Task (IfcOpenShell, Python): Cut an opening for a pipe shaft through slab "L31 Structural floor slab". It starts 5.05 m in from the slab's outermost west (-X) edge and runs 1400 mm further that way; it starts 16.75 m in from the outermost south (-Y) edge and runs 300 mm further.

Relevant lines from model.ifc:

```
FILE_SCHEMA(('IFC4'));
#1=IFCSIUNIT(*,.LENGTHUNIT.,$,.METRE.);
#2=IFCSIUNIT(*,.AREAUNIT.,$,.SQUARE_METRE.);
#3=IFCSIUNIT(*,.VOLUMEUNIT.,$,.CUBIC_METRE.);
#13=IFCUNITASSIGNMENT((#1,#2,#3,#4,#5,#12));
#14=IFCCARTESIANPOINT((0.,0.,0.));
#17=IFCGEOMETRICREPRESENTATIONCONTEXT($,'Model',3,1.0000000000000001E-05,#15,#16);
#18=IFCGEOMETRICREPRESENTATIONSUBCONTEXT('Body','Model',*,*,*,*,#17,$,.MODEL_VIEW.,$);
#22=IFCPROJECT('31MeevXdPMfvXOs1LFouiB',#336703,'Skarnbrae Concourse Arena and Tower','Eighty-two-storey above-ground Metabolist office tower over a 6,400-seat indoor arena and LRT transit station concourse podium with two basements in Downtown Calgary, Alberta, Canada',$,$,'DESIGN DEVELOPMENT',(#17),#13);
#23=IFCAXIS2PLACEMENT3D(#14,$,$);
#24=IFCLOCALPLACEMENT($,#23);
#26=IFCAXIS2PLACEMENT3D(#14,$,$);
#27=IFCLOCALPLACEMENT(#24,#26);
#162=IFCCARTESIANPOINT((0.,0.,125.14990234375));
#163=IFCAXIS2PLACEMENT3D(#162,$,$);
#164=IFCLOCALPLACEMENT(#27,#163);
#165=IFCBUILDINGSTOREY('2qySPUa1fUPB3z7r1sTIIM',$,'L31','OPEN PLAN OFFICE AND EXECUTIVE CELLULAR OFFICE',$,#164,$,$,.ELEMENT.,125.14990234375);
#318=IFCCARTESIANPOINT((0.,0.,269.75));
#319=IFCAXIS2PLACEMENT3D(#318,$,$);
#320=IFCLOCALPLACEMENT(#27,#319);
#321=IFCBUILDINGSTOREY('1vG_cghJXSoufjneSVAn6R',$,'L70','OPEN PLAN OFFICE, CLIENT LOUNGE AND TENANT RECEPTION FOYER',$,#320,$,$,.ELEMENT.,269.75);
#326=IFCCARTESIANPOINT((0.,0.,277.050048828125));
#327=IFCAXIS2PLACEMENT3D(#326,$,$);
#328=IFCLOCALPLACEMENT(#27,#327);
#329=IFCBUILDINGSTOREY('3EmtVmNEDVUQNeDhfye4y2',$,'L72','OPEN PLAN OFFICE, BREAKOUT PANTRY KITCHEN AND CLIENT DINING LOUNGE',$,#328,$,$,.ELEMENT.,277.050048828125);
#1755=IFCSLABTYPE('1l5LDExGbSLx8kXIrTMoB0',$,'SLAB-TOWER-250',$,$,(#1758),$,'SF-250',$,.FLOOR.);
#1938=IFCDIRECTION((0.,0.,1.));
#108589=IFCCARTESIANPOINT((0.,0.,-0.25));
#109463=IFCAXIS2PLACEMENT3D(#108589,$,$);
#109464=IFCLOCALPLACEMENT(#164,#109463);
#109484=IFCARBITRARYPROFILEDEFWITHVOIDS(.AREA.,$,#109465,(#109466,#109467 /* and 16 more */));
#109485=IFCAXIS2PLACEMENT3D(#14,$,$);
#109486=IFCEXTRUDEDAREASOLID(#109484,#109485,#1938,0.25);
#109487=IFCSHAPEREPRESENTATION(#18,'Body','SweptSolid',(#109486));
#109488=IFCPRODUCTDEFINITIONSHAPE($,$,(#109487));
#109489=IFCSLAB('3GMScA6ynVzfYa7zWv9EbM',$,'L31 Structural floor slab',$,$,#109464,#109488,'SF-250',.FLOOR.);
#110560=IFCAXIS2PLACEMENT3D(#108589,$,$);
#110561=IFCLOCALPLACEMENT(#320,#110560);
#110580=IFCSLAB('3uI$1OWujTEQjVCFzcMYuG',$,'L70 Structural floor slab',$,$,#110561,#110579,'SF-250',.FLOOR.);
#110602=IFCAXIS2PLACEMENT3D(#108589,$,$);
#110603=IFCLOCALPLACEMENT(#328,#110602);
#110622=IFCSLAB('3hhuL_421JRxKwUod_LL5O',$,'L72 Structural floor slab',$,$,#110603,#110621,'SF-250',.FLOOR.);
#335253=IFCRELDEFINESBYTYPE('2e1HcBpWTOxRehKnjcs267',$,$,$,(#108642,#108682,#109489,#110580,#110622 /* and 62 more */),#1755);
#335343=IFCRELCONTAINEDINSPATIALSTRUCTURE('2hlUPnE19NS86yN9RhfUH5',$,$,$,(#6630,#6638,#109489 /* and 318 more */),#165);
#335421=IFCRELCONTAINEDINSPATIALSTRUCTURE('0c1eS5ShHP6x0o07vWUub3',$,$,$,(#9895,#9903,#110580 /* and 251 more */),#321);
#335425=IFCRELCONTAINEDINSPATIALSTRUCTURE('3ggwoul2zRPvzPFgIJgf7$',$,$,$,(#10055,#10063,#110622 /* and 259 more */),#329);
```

```python
import numpy as np
import ifcopenshell
import ifcopenshell.api.feature
import ifcopenshell.api.geometry
import ifcopenshell.api.root
import ifcopenshell.geom
import ifcopenshell.util.placement
import ifcopenshell.util.representation
import ifcopenshell.util.shape
import ifcopenshell.util.unit

model = ifcopenshell.open("model.ifc")
unit_scale = ifcopenshell.util.unit.calculate_unit_scale(model)
settings = ifcopenshell.geom.settings()


def volume(element):
    """Net volume in cubic metres, openings subtracted."""
    shape = ifcopenshell.geom.create_shape(settings, element)
    return ifcopenshell.util.shape.get_volume(shape.geometry)


slab = model.by_id(109489)
before = volume(slab)

# Extent in the slab's own axes, in metres. The edges named are its -X and -Y sides.
slab_shape = ifcopenshell.geom.create_shape(settings, slab)
vertices = ifcopenshell.util.shape.get_vertices(slab_shape.geometry)
x_min, y_min, bottom = vertices.min(axis=0)
top = vertices[:, 2].max()

opening = ifcopenshell.api.root.create_entity(model, ifc_class="IfcOpeningElement", name="Pipe shaft opening", predefined_type="OPENING")
context = ifcopenshell.util.representation.get_context(model, "Model", "Body", "MODEL_VIEW")
width, depth = 1.4, 0.3
outline = [(0.0, 0.0), (width, 0.0), (width, depth), (0.0, depth), (0.0, 0.0)]
# Overshoot both faces by 50 mm so the cut is clean.
shape = ifcopenshell.api.geometry.add_slab_representation(
    model, context=context, depth=top - bottom + 0.1, polyline=outline
)
ifcopenshell.api.geometry.assign_representation(model, product=opening, representation=shape)

matrix = ifcopenshell.util.placement.get_local_placement(slab.ObjectPlacement)
matrix[:, 3] = matrix @ np.append(np.array([x_min + 5.05, y_min + 16.75, bottom - 0.05]) / unit_scale, 1.0)
ifcopenshell.api.geometry.edit_object_placement(model, product=opening, matrix=matrix, is_si=False)
ifcopenshell.api.feature.add_feature(model, feature=opening, element=slab)

after = volume(slab)

print(f"slab volume {before:.3f} -> {after:.3f} m3")

model.write("model_rev.ifc")
```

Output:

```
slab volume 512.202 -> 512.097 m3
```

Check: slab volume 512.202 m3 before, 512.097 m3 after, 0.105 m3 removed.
